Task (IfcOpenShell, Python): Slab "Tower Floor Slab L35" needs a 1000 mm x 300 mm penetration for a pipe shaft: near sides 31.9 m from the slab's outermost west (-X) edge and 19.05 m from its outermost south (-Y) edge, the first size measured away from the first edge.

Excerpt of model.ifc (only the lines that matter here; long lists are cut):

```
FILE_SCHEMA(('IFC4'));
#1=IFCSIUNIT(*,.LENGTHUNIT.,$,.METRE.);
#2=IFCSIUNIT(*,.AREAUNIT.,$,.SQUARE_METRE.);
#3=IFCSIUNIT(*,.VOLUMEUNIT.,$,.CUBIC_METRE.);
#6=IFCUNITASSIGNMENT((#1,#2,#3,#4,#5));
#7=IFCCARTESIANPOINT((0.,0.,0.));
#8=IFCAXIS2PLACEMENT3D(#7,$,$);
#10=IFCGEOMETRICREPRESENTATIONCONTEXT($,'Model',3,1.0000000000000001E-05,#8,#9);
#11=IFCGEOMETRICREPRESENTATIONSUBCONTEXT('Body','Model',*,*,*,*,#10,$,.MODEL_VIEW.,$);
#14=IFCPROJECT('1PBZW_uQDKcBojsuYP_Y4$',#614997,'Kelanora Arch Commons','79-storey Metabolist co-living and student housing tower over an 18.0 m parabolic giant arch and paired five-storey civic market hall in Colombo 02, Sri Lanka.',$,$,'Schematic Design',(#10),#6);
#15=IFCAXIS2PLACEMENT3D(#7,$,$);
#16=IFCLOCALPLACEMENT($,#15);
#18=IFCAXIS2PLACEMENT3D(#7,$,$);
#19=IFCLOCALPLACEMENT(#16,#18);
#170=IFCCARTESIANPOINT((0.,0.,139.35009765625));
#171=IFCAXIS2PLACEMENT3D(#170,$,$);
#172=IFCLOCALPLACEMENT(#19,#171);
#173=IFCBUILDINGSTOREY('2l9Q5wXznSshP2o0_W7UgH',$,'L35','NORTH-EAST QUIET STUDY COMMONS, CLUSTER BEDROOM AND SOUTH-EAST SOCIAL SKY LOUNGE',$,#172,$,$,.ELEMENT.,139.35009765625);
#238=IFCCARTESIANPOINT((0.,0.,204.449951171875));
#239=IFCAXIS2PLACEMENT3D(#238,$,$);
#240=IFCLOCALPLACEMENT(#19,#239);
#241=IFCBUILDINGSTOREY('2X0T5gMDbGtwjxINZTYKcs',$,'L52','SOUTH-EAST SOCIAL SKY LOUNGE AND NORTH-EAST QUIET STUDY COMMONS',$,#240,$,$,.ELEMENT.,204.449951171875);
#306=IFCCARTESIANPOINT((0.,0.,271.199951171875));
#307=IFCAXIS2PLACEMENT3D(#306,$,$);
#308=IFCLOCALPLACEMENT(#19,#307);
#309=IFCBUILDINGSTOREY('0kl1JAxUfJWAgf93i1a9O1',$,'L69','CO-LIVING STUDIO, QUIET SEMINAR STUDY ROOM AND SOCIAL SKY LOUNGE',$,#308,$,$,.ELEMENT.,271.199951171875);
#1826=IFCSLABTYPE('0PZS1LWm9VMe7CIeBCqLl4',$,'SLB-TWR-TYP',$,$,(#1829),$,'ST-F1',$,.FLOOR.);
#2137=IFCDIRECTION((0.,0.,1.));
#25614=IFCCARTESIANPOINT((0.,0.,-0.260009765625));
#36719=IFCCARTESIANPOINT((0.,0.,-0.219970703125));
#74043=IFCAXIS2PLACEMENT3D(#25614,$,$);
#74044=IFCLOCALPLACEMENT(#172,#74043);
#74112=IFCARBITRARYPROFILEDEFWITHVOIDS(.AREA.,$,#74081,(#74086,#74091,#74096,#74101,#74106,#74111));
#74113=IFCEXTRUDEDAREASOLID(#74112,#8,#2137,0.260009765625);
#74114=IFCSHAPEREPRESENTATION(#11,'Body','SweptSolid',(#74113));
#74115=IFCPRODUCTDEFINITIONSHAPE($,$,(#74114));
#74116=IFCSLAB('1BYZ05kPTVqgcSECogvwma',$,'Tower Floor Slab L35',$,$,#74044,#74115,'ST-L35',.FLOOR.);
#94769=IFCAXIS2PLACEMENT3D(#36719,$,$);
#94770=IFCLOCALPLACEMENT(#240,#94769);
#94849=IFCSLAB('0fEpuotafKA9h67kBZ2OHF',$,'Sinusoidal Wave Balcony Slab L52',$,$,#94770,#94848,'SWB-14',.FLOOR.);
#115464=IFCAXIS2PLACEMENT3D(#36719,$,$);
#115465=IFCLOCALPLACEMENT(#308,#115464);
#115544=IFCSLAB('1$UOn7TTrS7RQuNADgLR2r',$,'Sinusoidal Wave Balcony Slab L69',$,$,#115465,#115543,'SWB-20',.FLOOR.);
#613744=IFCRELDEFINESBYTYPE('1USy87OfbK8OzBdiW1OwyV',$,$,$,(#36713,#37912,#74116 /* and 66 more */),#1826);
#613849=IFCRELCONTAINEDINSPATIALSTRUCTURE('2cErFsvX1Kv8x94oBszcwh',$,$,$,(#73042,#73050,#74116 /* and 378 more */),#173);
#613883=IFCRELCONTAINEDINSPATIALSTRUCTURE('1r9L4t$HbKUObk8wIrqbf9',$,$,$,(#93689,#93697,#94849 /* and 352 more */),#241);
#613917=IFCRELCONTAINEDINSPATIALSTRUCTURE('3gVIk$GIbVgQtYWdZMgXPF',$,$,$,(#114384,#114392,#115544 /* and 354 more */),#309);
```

```python
import numpy as np
import ifcopenshell
import ifcopenshell.api.feature
import ifcopenshell.api.geometry
import ifcopenshell.api.root
import ifcopenshell.geom
import ifcopenshell.util.placement
import ifcopenshell.util.representation
import ifcopenshell.util.shape
import ifcopenshell.util.unit

model = ifcopenshell.open("model.ifc")
unit_scale = ifcopenshell.util.unit.calculate_unit_scale(model)
settings = ifcopenshell.geom.settings()


def volume(element):
    """Net volume in cubic metres, openings subtracted."""
    shape = ifcopenshell.geom.create_shape(settings, element)
    return ifcopenshell.util.shape.get_volume(shape.geometry)


slab = model.by_id(74116)
before = volume(slab)

# Extent in the slab's own axes, in metres. The edges named are its -X and -Y sides.
slab_shape = ifcopenshell.geom.create_shape(settings, slab)
vertices = ifcopenshell.util.shape.get_vertices(slab_shape.geometry)
x_min, y_min, bottom = vertices.min(axis=0)
top = vertices[:, 2].max()

opening = ifcopenshell.api.root.create_entity(model, ifc_class="IfcOpeningElement", name="Pipe shaft opening", predefined_type="OPENING")
context = ifcopenshell.util.representation.get_context(model, "Model", "Body", "MODEL_VIEW")
width, depth = 1, 0.3
outline = [(0.0, 0.0), (width, 0.0), (width, depth), (0.0, depth), (0.0, 0.0)]
# Overshoot both faces by 50 mm so the cut is clean.
shape = ifcopenshell.api.geometry.add_slab_representation(
    model, context=context, depth=top - bottom + 0.1, polyline=outline
)
ifcopenshell.api.geometry.assign_representation(model, product=opening, representation=shape)

matrix = ifcopenshell.util.placement.get_local_placement(slab.ObjectPlacement)
matrix[:, 3] = matrix @ np.append(np.array([x_min + 31.9, y_min + 19.05, bottom - 0.05]) / unit_scale, 1.0)
ifcopenshell.api.geometry.edit_object_placement(model, product=opening, matrix=matrix, is_si=False)
ifcopenshell.api.feature.add_feature(model, feature=opening, element=slab)

after = volume(slab)

print(f"slab volume {before:.3f} -> {after:.3f} m3")

model.write("model_v2.ifc")
```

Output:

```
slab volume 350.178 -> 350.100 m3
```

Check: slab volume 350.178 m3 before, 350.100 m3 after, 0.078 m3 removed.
